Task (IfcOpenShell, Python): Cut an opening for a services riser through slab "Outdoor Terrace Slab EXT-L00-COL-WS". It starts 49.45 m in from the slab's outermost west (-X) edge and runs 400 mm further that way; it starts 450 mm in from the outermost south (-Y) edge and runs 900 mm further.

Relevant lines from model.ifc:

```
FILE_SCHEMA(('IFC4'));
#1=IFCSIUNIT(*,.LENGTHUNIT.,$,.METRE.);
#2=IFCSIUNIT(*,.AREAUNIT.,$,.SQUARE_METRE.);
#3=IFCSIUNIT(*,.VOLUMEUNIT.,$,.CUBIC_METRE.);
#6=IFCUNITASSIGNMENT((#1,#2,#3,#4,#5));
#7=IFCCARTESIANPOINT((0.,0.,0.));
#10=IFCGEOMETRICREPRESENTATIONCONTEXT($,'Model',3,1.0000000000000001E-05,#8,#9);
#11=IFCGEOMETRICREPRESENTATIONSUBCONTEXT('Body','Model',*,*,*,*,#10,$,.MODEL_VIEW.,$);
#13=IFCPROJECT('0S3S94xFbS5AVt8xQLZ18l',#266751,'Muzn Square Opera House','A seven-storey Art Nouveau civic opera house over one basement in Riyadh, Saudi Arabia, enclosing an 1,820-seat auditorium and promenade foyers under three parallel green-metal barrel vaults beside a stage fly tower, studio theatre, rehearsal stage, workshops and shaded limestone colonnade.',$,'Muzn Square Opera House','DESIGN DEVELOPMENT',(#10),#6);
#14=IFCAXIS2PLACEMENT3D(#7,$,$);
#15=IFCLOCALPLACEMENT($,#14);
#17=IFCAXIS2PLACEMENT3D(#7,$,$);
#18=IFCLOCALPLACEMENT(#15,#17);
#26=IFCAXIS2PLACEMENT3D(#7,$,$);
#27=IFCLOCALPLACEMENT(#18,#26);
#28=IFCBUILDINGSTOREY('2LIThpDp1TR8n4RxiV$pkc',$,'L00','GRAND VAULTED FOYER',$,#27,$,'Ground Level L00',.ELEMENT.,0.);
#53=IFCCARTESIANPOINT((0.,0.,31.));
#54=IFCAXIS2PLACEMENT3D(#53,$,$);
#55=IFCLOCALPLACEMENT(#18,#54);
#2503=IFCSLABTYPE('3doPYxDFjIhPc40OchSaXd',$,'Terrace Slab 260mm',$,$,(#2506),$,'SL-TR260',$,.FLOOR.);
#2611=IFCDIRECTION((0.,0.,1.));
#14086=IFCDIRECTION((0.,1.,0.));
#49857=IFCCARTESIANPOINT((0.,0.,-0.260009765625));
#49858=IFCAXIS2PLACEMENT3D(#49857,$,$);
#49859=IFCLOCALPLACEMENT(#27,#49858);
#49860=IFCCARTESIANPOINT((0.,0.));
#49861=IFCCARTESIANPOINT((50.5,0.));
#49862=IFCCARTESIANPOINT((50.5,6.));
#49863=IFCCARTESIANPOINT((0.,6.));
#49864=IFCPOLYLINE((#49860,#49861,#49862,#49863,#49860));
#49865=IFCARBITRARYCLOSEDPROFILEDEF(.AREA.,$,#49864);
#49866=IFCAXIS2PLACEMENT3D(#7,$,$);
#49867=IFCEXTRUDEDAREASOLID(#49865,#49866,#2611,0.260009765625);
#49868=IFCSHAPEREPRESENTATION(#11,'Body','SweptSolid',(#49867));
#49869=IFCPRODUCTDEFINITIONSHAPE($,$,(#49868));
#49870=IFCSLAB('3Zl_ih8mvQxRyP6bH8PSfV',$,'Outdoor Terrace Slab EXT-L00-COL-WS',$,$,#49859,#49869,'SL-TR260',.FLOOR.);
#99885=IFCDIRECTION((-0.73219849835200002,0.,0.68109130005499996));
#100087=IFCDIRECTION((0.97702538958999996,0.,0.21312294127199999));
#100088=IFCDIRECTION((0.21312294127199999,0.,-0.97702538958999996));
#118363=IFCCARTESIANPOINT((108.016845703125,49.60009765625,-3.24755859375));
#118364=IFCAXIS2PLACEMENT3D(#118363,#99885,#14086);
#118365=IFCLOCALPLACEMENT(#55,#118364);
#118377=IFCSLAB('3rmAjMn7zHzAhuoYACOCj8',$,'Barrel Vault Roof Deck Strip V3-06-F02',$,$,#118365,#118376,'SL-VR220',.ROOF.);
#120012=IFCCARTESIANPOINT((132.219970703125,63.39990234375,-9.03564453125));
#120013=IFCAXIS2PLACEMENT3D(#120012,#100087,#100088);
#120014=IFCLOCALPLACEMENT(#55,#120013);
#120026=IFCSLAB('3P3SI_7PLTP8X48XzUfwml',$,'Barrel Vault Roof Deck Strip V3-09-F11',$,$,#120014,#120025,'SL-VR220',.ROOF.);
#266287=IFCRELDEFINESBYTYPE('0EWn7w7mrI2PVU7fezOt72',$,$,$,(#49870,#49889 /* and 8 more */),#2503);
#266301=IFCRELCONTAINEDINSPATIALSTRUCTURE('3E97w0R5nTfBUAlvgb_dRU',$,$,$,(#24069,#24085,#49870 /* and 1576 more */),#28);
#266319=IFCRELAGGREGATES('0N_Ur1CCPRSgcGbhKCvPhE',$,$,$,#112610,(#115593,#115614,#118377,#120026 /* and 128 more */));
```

```python
import numpy as np
import ifcopenshell
import ifcopenshell.api.feature
import ifcopenshell.api.geometry
import ifcopenshell.api.root
import ifcopenshell.geom
import ifcopenshell.util.placement
import ifcopenshell.util.representation
import ifcopenshell.util.shape
import ifcopenshell.util.unit

model = ifcopenshell.open("model.ifc")
unit_scale = ifcopenshell.util.unit.calculate_unit_scale(model)
settings = ifcopenshell.geom.settings()


def volume(element):
    """Net volume in cubic metres, openings subtracted."""
    shape = ifcopenshell.geom.create_shape(settings, element)
    return ifcopenshell.util.shape.get_volume(shape.geometry)


slab = model.by_guid("3Zl_ih8mvQxRyP6bH8PSfV")
before = volume(slab)

# Extent in the slab's own axes, in metres. The edges named are its -X and -Y sides.
slab_shape = ifcopenshell.geom.create_shape(settings, slab)
vertices = ifcopenshell.util.shape.get_vertices(slab_shape.geometry)
x_min, y_min, bottom = vertices.min(axis=0)
top = vertices[:, 2].max()

opening = ifcopenshell.api.root.create_entity(model, ifc_class="IfcOpeningElement", name="Services riser opening", predefined_type="OPENING")
context = ifcopenshell.util.representation.get_context(model, "Model", "Body", "MODEL_VIEW")
width, depth = 0.4, 0.9
outline = [(0.0, 0.0), (width, 0.0), (width, depth), (0.0, depth), (0.0, 0.0)]
# Overshoot both faces by 50 mm so the cut is clean.
shape = ifcopenshell.api.geometry.add_slab_representation(
    model, context=context, depth=top - bottom + 0.1, polyline=outline
)
ifcopenshell.api.geometry.assign_representation(model, product=opening, representation=shape)

matrix = ifcopenshell.util.placement.get_local_placement(slab.ObjectPlacement)
matrix[:, 3] = matrix @ np.append(np.array([x_min + 49.45, y_min + 0.45, bottom - 0.05]) / unit_scale, 1.0)
ifcopenshell.api.geometry.edit_object_placement(model, product=opening, matrix=matrix, is_si=False)
ifcopenshell.api.feature.add_feature(model, feature=opening, element=slab)

after = volume(slab)

print(f"slab volume {before:.3f} -> {after:.3f} m3")

model.write("model_rev.ifc")
```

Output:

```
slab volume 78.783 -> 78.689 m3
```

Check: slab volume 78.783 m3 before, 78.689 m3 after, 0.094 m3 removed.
